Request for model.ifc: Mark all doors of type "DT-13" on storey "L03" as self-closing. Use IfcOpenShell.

First a look at what the model holds.

```python
import ifcopenshell
import ifcopenshell.util.element

model = ifcopenshell.open("model.ifc")
print(model.schema)
storey = next(s for s in model.by_type("IfcBuildingStorey") if s.Name == "L03")
doors = [e for e in ifcopenshell.util.element.get_decomposition(storey) if e.is_a("IfcDoor")]
seen = {}
for e in doors:
    element_type = ifcopenshell.util.element.get_type(e)
    key = (element_type.Name if element_type != e and element_type else None, ifcopenshell.util.element.get_pset(e, "Pset_DoorCommon", "SelfClosing"))
    seen[key] = seen.get(key, 0) + 1
for (name, value), count in sorted(seen.items(), key=str):
    print(count, "x", name, "|", value)
```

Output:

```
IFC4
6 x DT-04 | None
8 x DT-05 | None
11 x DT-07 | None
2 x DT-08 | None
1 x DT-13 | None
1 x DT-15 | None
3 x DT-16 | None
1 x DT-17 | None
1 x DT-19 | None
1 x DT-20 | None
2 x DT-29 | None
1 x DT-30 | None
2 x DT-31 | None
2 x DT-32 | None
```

```python
import ifcopenshell
import ifcopenshell.api.pset
import ifcopenshell.util.element

model = ifcopenshell.open("model.ifc")

storey = next(s for s in model.by_type("IfcBuildingStorey") if s.Name == "L03")
doors = [e for e in ifcopenshell.util.element.get_decomposition(storey) if e.is_a("IfcDoor")]

count = 0
for e in doors:
    element_type = ifcopenshell.util.element.get_type(e)
    if element_type in (None, e) or element_type.Name != "DT-13":
        continue
    # add_pset returns the element's existing set when there is one.
    pset = ifcopenshell.api.pset.add_pset(model, product=e, name="Pset_DoorCommon")
    ifcopenshell.api.pset.edit_pset(model, pset=pset, properties={"SelfClosing": True})
    count += 1

print(count, "doors updated")

model.write("model_v2.ifc")
```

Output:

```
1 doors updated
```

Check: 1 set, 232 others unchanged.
